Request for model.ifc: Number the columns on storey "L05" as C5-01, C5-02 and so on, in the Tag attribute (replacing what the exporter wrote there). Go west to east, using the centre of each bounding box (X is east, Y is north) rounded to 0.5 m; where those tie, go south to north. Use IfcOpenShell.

First a look at what the model holds.

```python
import ifcopenshell
import ifcopenshell.util.element
import ifcopenshell.util.placement

model = ifcopenshell.open("model.ifc")
print(model.schema)
storey = next(s for s in model.by_type("IfcBuildingStorey") if s.Name == "L05")
columns = [e for e in ifcopenshell.util.element.get_decomposition(storey) if e.is_a("IfcColumn")]
for e in sorted(columns, key=lambda e: e.id()):
    origin = ifcopenshell.util.placement.get_local_placement(e.ObjectPlacement)[:3, 3]
    print(e.id(), e.Tag, e.Name, origin.round(2) + 0.0, sep=" | ")
```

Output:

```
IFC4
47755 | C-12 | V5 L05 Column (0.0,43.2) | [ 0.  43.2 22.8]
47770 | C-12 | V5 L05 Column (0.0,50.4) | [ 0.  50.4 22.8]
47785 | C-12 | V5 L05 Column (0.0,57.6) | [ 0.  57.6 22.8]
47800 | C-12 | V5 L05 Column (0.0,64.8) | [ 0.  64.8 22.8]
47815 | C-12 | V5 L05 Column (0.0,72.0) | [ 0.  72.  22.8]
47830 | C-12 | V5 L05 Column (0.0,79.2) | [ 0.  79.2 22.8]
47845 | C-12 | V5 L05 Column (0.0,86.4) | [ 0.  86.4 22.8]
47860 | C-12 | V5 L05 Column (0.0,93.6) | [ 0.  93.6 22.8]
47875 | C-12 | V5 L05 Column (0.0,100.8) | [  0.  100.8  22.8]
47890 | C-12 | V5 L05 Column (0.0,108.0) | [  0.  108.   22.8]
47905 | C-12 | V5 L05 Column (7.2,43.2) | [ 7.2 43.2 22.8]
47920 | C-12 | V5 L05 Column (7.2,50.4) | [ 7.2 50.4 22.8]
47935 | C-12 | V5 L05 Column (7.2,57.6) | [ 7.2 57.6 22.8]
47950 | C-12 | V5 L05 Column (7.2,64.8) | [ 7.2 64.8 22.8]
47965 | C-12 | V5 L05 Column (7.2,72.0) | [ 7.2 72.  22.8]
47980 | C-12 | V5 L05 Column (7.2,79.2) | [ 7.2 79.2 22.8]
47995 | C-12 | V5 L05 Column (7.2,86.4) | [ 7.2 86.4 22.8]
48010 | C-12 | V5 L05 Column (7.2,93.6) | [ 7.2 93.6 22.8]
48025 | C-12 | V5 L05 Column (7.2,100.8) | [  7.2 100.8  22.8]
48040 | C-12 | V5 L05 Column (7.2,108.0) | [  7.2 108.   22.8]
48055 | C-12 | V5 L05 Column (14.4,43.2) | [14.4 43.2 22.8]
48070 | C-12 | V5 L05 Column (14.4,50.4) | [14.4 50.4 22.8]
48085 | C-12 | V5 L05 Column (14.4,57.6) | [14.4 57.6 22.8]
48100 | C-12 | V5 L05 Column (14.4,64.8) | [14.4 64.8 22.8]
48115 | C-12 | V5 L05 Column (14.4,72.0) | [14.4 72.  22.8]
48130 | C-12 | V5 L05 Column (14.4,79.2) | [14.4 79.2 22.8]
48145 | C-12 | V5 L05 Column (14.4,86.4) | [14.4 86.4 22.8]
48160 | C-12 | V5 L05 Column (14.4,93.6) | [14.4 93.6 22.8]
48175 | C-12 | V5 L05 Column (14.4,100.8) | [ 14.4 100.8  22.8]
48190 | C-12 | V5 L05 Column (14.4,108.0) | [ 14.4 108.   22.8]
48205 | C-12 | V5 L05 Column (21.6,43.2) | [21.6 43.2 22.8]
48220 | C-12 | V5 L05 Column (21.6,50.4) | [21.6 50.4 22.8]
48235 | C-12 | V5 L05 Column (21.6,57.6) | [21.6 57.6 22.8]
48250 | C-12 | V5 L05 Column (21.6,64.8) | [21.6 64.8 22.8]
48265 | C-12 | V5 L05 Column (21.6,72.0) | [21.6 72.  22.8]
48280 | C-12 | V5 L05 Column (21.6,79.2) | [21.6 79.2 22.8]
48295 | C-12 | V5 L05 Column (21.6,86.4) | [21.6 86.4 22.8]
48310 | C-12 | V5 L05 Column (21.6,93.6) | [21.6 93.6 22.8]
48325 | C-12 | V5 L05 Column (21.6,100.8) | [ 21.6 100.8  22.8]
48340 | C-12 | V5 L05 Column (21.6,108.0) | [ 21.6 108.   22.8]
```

```python
import ifcopenshell
import ifcopenshell.geom
import ifcopenshell.util.element
import ifcopenshell.util.shape

model = ifcopenshell.open("model.ifc")
settings = ifcopenshell.geom.settings()
settings.set("use-world-coords", True)


def centre(element):
    shape = ifcopenshell.geom.create_shape(settings, element)
    return ifcopenshell.util.shape.get_bbox_centroid(shape.geometry)


storey = next(s for s in model.by_type("IfcBuildingStorey") if s.Name == "L05")
columns = [e for e in ifcopenshell.util.element.get_decomposition(storey) if e.is_a("IfcColumn")]

# Insertion points can sit at a corner or the storey origin, so sort by the geometry (in metres).
centres = {e: centre(e) for e in columns}
columns.sort(key=lambda e: (round(centres[e][0] / 0.5), centres[e][1]))

for i, e in enumerate(columns, start=1):
    number = f"C5-{i:02d}"
    e.Tag = number
    print(e.id(), number)

model.write("model_updated.ifc")
```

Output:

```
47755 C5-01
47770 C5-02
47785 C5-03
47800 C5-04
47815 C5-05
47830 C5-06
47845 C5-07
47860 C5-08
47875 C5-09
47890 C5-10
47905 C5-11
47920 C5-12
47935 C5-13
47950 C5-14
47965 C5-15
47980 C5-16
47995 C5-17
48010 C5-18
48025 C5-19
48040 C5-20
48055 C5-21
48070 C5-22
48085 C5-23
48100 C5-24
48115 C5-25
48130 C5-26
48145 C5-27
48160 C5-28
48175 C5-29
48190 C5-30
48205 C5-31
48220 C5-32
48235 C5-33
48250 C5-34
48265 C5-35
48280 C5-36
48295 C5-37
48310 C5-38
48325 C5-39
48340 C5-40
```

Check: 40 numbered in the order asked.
